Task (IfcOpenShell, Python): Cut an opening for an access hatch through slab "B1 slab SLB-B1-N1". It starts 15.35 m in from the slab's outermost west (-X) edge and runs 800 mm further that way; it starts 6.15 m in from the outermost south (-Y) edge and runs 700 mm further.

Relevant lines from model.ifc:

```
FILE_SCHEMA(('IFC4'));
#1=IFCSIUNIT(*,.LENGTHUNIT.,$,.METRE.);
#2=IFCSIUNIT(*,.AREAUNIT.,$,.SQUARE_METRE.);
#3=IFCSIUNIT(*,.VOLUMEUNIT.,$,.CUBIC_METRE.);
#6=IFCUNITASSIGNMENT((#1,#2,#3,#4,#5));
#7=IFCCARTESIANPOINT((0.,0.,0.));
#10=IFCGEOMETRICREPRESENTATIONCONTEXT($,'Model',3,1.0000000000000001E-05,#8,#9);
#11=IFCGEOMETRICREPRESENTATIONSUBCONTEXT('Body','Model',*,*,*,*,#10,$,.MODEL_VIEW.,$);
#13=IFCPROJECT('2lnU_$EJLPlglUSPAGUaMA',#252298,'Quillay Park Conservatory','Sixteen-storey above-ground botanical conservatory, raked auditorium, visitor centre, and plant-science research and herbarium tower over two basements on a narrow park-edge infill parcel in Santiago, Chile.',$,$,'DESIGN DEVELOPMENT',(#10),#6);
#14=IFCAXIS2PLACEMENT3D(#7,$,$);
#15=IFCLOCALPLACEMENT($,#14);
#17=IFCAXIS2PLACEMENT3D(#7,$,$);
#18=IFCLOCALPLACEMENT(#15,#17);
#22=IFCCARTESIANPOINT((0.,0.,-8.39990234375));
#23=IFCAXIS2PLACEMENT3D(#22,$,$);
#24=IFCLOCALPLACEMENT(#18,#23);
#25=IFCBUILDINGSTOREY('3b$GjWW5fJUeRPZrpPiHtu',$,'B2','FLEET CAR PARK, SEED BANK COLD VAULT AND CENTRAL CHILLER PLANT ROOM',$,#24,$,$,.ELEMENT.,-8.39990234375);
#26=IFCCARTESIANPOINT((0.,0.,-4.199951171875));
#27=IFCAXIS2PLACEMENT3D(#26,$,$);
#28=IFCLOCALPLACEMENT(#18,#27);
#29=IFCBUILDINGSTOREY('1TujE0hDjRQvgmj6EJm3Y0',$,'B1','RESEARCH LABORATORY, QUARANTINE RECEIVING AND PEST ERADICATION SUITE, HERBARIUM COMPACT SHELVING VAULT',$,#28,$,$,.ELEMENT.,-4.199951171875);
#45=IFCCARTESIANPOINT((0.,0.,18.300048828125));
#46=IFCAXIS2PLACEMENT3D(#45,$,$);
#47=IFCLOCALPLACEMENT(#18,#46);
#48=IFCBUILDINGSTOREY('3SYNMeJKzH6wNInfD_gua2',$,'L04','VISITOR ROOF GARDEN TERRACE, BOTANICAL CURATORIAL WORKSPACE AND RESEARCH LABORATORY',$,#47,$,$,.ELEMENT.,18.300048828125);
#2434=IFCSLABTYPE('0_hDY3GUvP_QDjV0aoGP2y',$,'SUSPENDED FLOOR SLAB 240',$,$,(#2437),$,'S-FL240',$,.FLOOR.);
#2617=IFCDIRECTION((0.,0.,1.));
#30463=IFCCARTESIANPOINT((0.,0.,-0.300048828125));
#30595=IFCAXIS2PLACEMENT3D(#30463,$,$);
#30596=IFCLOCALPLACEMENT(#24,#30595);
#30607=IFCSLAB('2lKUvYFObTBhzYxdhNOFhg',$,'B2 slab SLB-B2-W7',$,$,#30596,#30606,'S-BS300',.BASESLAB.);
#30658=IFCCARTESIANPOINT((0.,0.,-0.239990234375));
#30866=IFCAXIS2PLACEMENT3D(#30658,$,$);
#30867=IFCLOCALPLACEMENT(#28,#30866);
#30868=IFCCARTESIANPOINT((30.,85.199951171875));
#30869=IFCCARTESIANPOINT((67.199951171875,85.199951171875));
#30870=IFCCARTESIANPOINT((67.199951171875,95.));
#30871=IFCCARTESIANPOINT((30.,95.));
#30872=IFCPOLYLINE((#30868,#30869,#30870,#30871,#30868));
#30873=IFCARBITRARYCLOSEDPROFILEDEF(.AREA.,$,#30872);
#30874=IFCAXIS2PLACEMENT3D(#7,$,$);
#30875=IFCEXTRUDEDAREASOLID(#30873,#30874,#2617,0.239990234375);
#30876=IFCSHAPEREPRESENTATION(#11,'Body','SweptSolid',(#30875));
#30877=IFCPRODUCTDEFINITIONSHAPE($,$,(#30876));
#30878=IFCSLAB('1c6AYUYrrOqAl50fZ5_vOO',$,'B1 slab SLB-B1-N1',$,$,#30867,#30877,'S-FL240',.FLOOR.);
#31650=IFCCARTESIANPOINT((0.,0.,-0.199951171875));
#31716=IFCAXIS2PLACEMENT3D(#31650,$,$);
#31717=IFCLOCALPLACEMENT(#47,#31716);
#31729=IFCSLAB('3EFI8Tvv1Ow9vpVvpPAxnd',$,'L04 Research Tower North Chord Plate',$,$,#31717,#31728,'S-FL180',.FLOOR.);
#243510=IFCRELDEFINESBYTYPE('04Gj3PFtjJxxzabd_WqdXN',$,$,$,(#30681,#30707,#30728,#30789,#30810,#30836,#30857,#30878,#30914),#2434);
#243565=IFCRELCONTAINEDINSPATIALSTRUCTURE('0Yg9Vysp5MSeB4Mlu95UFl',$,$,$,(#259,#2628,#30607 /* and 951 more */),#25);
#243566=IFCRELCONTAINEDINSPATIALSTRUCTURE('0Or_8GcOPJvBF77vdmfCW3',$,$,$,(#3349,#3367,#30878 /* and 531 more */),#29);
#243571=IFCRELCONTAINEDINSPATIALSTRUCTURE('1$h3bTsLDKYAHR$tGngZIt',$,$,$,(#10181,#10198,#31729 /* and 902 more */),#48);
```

```python
import numpy as np
import ifcopenshell
import ifcopenshell.api.feature
import ifcopenshell.api.geometry
import ifcopenshell.api.root
import ifcopenshell.geom
import ifcopenshell.util.placement
import ifcopenshell.util.representation
import ifcopenshell.util.shape
import ifcopenshell.util.unit

model = ifcopenshell.open("model.ifc")
unit_scale = ifcopenshell.util.unit.calculate_unit_scale(model)
settings = ifcopenshell.geom.settings()


def volume(element):
    """Net volume in cubic metres, openings subtracted."""
    shape = ifcopenshell.geom.create_shape(settings, element)
    return ifcopenshell.util.shape.get_volume(shape.geometry)


slab = model.by_id(30878)
before = volume(slab)

# Extent in the slab's own axes, in metres. The edges named are its -X and -Y sides.
slab_shape = ifcopenshell.geom.create_shape(settings, slab)
vertices = ifcopenshell.util.shape.get_vertices(slab_shape.geometry)
x_min, y_min, bottom = vertices.min(axis=0)
top = vertices[:, 2].max()

opening = ifcopenshell.api.root.create_entity(model, ifc_class="IfcOpeningElement", name="Access hatch opening", predefined_type="OPENING")
context = ifcopenshell.util.representation.get_context(model, "Model", "Body", "MODEL_VIEW")
width, depth = 0.8, 0.7
outline = [(0.0, 0.0), (width, 0.0), (width, depth), (0.0, depth), (0.0, 0.0)]
# Overshoot both faces by 50 mm so the cut is clean.
shape = ifcopenshell.api.geometry.add_slab_representation(
    model, context=context, depth=top - bottom + 0.1, polyline=outline
)
ifcopenshell.api.geometry.assign_representation(model, product=opening, representation=shape)

matrix = ifcopenshell.util.placement.get_local_placement(slab.ObjectPlacement)
matrix[:, 3] = matrix @ np.append(np.array([x_min + 15.35, y_min + 6.15, bottom - 0.05]) / unit_scale, 1.0)
ifcopenshell.api.geometry.edit_object_placement(model, product=opening, matrix=matrix, is_si=False)
ifcopenshell.api.feature.add_feature(model, feature=opening, element=slab)

after = volume(slab)

print(f"slab volume {before:.3f} -> {after:.3f} m3")

model.write("model_rev.ifc")
```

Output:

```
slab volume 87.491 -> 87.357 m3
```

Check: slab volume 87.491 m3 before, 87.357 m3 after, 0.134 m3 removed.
